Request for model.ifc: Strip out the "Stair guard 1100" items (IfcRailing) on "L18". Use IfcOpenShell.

First a look at what the model holds.

```python
import ifcopenshell
import ifcopenshell.util.element

model = ifcopenshell.open("model.ifc")
print(model.schema)
storey = next(s for s in model.by_type("IfcBuildingStorey") if s.Name == "L18")
railings = [e for e in ifcopenshell.util.element.get_decomposition(storey) if e.is_a("IfcRailing")]
seen = {}
for e in railings:
    element_type = ifcopenshell.util.element.get_type(e)
    name = element_type.Name if element_type not in (None, e) else None
    seen[name] = seen.get(name, 0) + 1
for name, count in sorted(seen.items(), key=str):
    print(count, "x", name)
```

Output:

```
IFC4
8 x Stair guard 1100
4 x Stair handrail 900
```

```python
import ifcopenshell
import ifcopenshell.api.root
import ifcopenshell.util.element

model = ifcopenshell.open("model.ifc")

storey = next(s for s in model.by_type("IfcBuildingStorey") if s.Name == "L18")
railings = [e for e in ifcopenshell.util.element.get_decomposition(storey) if e.is_a("IfcRailing")]
targets = [e for e in railings if (t := ifcopenshell.util.element.get_type(e)) not in (None, e) and t.Name == "Stair guard 1100"]

for e in targets:
    ifcopenshell.api.root.remove_product(model, product=e)
print(len(targets), "removed")

model.write("model_edited.ifc")
```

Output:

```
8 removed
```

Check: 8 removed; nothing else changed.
